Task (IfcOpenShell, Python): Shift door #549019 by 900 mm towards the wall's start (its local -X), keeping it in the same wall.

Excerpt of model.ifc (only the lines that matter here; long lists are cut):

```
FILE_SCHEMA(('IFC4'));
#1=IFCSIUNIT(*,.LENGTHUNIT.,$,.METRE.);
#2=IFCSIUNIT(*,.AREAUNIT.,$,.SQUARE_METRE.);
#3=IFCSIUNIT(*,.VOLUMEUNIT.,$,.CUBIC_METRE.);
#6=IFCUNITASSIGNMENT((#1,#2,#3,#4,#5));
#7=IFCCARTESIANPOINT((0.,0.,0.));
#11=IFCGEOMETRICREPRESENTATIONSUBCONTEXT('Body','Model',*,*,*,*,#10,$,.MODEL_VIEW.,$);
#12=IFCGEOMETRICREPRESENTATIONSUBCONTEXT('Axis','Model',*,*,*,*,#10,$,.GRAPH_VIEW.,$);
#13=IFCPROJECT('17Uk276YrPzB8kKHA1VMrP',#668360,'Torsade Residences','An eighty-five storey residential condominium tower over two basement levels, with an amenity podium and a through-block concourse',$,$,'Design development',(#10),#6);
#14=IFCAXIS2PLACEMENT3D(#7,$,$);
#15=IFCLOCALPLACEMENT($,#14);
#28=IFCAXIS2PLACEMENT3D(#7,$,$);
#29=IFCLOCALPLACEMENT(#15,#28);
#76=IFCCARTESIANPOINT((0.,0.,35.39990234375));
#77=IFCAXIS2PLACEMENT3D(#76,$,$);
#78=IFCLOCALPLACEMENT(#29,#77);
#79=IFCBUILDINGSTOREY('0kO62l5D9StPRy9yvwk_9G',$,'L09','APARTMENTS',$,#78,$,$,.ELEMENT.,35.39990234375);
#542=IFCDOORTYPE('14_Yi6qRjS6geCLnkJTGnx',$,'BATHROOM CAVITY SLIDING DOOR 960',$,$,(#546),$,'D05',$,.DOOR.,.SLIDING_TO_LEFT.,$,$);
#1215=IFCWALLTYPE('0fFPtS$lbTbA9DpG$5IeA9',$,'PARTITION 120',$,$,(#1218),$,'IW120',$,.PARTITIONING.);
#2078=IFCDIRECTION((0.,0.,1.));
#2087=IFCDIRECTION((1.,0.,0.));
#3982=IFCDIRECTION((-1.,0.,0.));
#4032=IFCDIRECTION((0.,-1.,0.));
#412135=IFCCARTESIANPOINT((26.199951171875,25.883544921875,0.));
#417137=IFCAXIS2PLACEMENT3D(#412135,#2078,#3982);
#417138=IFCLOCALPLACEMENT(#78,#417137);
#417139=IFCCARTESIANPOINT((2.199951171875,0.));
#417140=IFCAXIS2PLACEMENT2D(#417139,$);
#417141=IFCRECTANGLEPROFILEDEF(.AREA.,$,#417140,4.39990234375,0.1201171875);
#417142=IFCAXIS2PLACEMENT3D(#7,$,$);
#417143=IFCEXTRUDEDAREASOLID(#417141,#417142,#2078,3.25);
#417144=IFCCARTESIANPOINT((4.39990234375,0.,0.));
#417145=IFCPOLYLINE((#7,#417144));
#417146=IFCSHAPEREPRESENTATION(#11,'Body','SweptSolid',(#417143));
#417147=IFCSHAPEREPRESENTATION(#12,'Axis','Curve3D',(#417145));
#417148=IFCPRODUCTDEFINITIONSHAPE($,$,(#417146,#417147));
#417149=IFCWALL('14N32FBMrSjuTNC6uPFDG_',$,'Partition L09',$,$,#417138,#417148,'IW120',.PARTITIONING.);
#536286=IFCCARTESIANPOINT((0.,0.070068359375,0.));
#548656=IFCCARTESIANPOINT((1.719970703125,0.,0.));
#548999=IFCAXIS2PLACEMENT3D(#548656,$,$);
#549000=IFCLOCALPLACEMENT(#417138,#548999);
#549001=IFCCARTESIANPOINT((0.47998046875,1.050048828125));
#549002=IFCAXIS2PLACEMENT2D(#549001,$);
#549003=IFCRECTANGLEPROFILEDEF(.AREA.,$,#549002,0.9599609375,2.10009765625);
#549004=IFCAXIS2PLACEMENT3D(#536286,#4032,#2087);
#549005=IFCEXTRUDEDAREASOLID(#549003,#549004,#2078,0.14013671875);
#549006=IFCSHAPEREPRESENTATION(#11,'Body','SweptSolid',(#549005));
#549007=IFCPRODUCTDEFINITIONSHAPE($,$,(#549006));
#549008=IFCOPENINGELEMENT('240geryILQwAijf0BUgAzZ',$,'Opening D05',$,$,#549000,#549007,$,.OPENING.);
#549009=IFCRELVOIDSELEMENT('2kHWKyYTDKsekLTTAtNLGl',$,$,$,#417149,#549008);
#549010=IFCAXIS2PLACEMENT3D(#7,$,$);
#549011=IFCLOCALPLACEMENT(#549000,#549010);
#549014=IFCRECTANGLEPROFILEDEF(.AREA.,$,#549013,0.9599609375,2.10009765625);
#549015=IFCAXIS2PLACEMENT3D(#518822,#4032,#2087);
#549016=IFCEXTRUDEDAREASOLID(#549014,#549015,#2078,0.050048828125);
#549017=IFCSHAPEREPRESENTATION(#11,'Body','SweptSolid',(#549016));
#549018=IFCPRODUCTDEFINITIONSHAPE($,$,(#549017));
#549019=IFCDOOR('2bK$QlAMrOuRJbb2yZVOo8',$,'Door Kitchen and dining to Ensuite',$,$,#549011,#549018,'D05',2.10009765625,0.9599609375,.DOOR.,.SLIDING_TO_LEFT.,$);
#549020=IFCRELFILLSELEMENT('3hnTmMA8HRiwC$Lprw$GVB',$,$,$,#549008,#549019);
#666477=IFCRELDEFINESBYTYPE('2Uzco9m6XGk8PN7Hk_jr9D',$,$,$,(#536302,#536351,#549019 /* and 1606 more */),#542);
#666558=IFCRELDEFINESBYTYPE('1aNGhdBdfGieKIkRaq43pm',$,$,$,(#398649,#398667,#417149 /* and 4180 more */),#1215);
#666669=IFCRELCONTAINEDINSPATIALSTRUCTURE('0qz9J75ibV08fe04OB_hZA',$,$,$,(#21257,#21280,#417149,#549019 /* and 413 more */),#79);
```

```python
import ifcopenshell
import ifcopenshell.api.geometry
import ifcopenshell.util.placement

model = ifcopenshell.open("model.ifc")

door = model.by_guid("2bK$QlAMrOuRJbb2yZVOo8")
opening = door.FillsVoids[0].RelatingOpeningElement
wall = opening.VoidsElements[0].RelatingBuildingElement

wall_matrix = ifcopenshell.util.placement.get_local_placement(wall.ObjectPlacement)
shift = wall_matrix[:3, 0] * -0.9
before = ifcopenshell.util.placement.get_local_placement(door.ObjectPlacement)[:3, 3].copy()

# The door is placed relative to its opening, so it follows when the opening moves.
matrix = ifcopenshell.util.placement.get_local_placement(opening.ObjectPlacement)
matrix[:3, 3] += shift
ifcopenshell.api.geometry.edit_object_placement(
    model, product=opening, matrix=matrix, is_si=False, should_transform_children=True
)

after = ifcopenshell.util.placement.get_local_placement(door.ObjectPlacement)[:3, 3]
print("door moved by", (after - before).round(3) + 0.0)

model.write("model_edited.ifc")
```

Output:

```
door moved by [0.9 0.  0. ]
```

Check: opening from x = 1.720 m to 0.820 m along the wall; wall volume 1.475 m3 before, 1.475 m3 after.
